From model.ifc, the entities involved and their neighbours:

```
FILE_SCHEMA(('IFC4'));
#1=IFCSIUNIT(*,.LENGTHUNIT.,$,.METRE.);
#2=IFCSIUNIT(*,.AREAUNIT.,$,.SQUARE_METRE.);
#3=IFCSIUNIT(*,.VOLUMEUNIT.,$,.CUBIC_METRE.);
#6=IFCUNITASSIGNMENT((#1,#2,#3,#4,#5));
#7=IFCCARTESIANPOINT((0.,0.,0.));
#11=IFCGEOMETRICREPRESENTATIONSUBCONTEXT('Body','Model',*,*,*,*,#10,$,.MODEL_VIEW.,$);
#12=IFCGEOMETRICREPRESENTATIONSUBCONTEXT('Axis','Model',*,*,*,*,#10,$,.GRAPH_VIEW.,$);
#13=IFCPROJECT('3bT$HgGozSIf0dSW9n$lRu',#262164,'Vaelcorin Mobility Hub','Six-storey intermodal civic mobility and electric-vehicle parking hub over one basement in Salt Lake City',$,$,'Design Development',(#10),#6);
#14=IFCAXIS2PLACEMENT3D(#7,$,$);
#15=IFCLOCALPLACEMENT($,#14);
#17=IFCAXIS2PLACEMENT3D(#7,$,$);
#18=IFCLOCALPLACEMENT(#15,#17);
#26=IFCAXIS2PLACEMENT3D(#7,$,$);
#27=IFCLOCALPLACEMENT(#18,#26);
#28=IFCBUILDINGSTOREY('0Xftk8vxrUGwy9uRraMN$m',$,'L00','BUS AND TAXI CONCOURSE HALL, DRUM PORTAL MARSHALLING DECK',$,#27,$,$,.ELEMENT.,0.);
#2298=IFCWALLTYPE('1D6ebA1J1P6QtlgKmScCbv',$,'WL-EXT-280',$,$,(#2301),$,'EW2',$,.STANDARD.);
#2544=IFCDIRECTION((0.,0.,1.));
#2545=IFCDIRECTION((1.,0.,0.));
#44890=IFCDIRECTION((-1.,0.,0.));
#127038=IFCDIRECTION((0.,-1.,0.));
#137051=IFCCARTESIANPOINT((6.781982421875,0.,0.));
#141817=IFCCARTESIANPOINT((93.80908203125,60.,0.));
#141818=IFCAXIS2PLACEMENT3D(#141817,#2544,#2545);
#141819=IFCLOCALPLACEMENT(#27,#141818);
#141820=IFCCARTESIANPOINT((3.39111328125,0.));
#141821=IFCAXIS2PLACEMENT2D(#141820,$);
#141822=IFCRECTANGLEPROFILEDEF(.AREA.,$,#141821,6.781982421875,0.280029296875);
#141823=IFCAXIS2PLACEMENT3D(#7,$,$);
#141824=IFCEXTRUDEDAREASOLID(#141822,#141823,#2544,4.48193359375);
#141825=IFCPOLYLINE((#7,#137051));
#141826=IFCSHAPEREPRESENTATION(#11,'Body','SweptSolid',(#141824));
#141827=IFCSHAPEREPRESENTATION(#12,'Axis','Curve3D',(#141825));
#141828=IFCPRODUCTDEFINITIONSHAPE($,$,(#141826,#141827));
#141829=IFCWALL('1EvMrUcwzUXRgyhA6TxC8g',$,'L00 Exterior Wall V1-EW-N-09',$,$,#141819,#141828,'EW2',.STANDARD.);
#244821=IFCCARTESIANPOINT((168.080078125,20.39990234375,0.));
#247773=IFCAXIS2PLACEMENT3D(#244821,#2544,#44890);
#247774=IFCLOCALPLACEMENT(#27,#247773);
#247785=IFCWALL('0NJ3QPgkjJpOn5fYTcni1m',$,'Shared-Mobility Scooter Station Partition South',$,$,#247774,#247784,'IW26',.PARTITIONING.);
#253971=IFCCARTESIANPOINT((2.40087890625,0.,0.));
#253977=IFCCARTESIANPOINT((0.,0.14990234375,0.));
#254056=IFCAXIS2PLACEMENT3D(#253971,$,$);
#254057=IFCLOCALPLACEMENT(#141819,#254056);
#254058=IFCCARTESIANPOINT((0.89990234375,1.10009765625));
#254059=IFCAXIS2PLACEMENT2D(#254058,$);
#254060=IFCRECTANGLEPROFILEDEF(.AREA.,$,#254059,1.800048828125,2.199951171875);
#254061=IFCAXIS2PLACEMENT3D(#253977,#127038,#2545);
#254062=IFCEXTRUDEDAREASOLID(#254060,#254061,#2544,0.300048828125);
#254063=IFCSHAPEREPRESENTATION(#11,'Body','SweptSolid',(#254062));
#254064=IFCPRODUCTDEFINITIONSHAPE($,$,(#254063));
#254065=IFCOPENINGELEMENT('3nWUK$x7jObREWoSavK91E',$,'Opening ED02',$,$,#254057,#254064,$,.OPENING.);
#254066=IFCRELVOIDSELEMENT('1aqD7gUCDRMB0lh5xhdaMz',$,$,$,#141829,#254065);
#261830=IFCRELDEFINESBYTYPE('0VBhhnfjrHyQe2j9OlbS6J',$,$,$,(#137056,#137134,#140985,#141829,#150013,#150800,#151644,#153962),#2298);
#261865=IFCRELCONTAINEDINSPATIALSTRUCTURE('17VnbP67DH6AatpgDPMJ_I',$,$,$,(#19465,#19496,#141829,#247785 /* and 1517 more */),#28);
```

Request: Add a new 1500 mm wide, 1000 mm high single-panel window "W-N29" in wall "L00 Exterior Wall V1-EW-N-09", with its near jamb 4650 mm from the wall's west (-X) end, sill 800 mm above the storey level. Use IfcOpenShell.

```python
import numpy as np
import ifcopenshell
import ifcopenshell.api.feature
import ifcopenshell.api.geometry
import ifcopenshell.api.root
import ifcopenshell.api.spatial
import ifcopenshell.geom
import ifcopenshell.util.element
import ifcopenshell.util.placement
import ifcopenshell.util.representation
import ifcopenshell.util.shape
import ifcopenshell.util.unit

model = ifcopenshell.open("model.ifc")
unit_scale = ifcopenshell.util.unit.calculate_unit_scale(model)
settings = ifcopenshell.geom.settings()


def volume(element):
    """Net volume in cubic metres, openings subtracted."""
    shape = ifcopenshell.geom.create_shape(settings, element)
    return ifcopenshell.util.shape.get_volume(shape.geometry)


wall = model.by_guid("1EvMrUcwzUXRgyhA6TxC8g")
storey = ifcopenshell.util.element.get_container(wall, ifc_class="IfcBuildingStorey")
context = ifcopenshell.util.representation.get_context(model, "Model", "Body", "MODEL_VIEW")
before = volume(wall)

width, height, from_end, sill = 1.5, 1, 4.65, 0.8  # metres

# The wall runs along its own X axis, and the end named is its -X end.
wall_shape = ifcopenshell.geom.create_shape(settings, wall)
x, y, z = ifcopenshell.util.shape.get_vertices(wall_shape.geometry).T
start = x.min() + from_end
face, thickness = float(y.min()), float(y.max() - y.min())
wall_matrix = ifcopenshell.util.placement.get_local_placement(wall.ObjectPlacement)
level = ifcopenshell.util.placement.get_local_placement(storey.ObjectPlacement)[2, 3]


def in_wall(x, y):
    """Placement at x, y metres in the wall's axes, at sill height."""
    matrix = wall_matrix.copy()
    matrix[:, 3] = wall_matrix @ np.array([x / unit_scale, y / unit_scale, 0.0, 1.0])
    matrix[2, 3] = level + sill / unit_scale
    return matrix


# Opening: a box that overshoots both wall faces by 50 mm.
opening = ifcopenshell.api.root.create_entity(model, ifc_class="IfcOpeningElement", predefined_type="OPENING")
box = ifcopenshell.api.geometry.add_wall_representation(
    model, context=context, length=width, height=height, thickness=thickness + 0.1
)
ifcopenshell.api.geometry.assign_representation(model, product=opening, representation=box)
ifcopenshell.api.geometry.edit_object_placement(model, product=opening, matrix=in_wall(start, face - 0.05), is_si=False)
ifcopenshell.api.feature.add_feature(model, feature=opening, element=wall)

window = ifcopenshell.api.root.create_entity(model, ifc_class="IfcWindow", name="W-N29", predefined_type="WINDOW")
window.OverallWidth, window.OverallHeight = width / unit_scale, height / unit_scale
window.PartitioningType = "SINGLE_PANEL"
body = ifcopenshell.api.geometry.add_window_representation(
    model,
    context=context,
    overall_width=window.OverallWidth,
    overall_height=window.OverallHeight,
    partition_type="SINGLE_PANEL",
)
ifcopenshell.api.geometry.assign_representation(model, product=window, representation=body)
ifcopenshell.api.spatial.assign_container(model, products=[window], relating_structure=storey)
ifcopenshell.api.feature.add_filling(model, opening=opening, element=window)

# Centre the window in the wall's thickness.
ifcopenshell.api.geometry.edit_object_placement(model, product=window, matrix=in_wall(start, face), is_si=False)
window_shape = ifcopenshell.geom.create_shape(settings, window)
depth = ifcopenshell.util.shape.get_vertices(window_shape.geometry)[:, 1]
offset = face + thickness / 2 - (depth.min() + depth.max()) / 2
ifcopenshell.api.geometry.edit_object_placement(model, product=window, matrix=in_wall(start, offset), is_si=False)

after = volume(wall)

print(f"wall volume {before:.3f} -> {after:.3f} m3")

model.write("model_rev.ifc")
```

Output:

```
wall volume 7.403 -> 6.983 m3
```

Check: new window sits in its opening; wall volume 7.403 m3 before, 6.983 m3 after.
